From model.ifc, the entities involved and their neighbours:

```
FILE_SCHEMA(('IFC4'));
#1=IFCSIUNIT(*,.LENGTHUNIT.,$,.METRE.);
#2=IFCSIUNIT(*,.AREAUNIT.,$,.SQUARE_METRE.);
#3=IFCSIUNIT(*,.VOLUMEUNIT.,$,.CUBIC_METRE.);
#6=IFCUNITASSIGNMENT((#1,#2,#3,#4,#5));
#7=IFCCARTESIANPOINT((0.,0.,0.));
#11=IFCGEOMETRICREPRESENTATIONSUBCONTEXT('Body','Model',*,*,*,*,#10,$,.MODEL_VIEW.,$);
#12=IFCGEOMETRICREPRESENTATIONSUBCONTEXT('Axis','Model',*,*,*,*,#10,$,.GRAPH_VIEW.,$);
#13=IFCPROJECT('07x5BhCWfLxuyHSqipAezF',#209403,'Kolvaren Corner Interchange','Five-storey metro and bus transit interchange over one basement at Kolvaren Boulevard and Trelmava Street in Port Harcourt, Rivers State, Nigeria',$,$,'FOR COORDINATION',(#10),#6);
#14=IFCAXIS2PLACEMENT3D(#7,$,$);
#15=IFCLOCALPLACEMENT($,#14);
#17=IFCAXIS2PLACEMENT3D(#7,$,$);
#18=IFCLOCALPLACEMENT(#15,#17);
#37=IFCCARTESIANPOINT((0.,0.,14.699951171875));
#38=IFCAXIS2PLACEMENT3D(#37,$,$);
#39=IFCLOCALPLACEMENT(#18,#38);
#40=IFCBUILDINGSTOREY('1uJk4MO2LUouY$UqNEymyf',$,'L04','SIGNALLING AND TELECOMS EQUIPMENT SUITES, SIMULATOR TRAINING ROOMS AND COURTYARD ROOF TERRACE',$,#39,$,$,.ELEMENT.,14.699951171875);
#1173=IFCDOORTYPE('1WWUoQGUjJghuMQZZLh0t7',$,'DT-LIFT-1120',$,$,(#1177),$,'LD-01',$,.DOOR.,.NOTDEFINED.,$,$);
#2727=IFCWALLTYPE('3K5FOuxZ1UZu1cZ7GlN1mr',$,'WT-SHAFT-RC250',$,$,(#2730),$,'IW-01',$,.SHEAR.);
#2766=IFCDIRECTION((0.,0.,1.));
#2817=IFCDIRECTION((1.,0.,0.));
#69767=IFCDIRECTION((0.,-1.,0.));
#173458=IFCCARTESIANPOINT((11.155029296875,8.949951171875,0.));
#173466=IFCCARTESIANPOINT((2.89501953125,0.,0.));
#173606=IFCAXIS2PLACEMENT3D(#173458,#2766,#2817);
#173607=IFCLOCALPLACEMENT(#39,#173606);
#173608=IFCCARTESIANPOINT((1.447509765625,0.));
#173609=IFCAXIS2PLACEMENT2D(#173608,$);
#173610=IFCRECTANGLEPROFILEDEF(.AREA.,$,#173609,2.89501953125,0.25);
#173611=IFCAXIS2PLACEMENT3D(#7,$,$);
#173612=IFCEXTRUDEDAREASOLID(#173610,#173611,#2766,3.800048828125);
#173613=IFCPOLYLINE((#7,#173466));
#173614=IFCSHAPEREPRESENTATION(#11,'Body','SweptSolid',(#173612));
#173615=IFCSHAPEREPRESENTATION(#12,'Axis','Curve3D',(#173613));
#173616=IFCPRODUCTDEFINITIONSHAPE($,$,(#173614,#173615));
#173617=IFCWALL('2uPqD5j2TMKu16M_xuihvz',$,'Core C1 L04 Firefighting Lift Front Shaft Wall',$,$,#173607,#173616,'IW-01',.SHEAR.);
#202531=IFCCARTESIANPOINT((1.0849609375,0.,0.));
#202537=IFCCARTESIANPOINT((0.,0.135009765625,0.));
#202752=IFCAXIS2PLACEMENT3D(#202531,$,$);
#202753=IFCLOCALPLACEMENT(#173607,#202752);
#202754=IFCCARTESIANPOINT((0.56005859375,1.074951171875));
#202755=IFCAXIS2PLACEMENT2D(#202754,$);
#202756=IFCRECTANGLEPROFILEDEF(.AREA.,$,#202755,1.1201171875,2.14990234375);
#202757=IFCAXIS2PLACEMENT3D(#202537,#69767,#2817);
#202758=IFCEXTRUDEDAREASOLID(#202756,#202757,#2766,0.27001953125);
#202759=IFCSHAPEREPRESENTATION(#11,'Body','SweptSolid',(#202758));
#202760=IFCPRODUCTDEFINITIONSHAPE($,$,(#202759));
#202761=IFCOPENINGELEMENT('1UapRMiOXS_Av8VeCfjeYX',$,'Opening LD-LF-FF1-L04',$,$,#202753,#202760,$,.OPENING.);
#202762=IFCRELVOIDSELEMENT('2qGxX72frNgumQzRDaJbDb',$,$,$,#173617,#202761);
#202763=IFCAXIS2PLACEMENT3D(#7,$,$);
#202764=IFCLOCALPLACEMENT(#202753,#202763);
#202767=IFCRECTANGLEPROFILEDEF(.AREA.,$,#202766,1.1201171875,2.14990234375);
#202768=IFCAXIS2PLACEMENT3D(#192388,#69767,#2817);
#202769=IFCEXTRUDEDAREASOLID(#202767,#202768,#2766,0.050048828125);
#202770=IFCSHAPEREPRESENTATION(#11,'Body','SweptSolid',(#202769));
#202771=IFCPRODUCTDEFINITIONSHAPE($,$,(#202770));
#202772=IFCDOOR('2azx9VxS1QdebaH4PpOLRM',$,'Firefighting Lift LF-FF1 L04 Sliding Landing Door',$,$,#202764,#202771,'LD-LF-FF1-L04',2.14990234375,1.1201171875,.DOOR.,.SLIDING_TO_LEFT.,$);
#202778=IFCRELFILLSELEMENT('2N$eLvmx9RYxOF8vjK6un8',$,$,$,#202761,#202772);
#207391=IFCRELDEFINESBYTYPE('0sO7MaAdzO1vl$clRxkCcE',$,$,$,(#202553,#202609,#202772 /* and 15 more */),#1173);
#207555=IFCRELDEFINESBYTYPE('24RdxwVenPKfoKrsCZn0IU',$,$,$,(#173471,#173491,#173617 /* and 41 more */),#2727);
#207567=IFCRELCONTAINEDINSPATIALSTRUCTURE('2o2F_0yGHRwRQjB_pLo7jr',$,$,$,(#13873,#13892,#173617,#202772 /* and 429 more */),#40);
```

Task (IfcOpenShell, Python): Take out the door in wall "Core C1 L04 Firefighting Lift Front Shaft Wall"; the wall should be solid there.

```python
import ifcopenshell
import ifcopenshell.api.feature
import ifcopenshell.api.root
import ifcopenshell.geom
import ifcopenshell.util.shape

model = ifcopenshell.open("model.ifc")
settings = ifcopenshell.geom.settings()


def volume(element):
    """Net volume in cubic metres, openings subtracted."""
    shape = ifcopenshell.geom.create_shape(settings, element)
    return ifcopenshell.util.shape.get_volume(shape.geometry)


door = model.by_id(202772)
opening = door.FillsVoids[0].RelatingOpeningElement
wall = opening.VoidsElements[0].RelatingBuildingElement
before = volume(wall)

ifcopenshell.api.root.remove_product(model, product=door)
ifcopenshell.api.feature.remove_feature(model, feature=opening)

after = volume(wall)

print(f"wall volume {before:.3f} -> {after:.3f} m3")

model.write("model_rev.ifc")
```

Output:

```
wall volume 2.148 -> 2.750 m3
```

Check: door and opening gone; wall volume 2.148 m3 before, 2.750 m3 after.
